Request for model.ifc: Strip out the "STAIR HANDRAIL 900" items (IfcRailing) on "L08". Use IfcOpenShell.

First a look at what the model holds.

```python
import ifcopenshell
import ifcopenshell.util.element

model = ifcopenshell.open("model.ifc")
print(model.schema)
storey = next(s for s in model.by_type("IfcBuildingStorey") if s.Name == "L08")
railings = [e for e in ifcopenshell.util.element.get_decomposition(storey) if e.is_a("IfcRailing")]
seen = {}
for e in railings:
    element_type = ifcopenshell.util.element.get_type(e)
    name = element_type.Name if element_type not in (None, e) else None
    seen[name] = seen.get(name, 0) + 1
for name, count in sorted(seen.items(), key=str):
    print(count, "x", name)
```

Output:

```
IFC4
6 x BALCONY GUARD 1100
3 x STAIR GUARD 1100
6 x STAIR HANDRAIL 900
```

```python
import ifcopenshell
import ifcopenshell.api.root
import ifcopenshell.util.element

model = ifcopenshell.open("model.ifc")

storey = next(s for s in model.by_type("IfcBuildingStorey") if s.Name == "L08")
railings = [e for e in ifcopenshell.util.element.get_decomposition(storey) if e.is_a("IfcRailing")]
targets = [e for e in railings if (t := ifcopenshell.util.element.get_type(e)) not in (None, e) and t.Name == "STAIR HANDRAIL 900"]

for e in targets:
    ifcopenshell.api.root.remove_product(model, product=e)
print(len(targets), "removed")

model.write("model-out.ifc")
```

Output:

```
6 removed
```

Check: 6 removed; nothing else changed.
